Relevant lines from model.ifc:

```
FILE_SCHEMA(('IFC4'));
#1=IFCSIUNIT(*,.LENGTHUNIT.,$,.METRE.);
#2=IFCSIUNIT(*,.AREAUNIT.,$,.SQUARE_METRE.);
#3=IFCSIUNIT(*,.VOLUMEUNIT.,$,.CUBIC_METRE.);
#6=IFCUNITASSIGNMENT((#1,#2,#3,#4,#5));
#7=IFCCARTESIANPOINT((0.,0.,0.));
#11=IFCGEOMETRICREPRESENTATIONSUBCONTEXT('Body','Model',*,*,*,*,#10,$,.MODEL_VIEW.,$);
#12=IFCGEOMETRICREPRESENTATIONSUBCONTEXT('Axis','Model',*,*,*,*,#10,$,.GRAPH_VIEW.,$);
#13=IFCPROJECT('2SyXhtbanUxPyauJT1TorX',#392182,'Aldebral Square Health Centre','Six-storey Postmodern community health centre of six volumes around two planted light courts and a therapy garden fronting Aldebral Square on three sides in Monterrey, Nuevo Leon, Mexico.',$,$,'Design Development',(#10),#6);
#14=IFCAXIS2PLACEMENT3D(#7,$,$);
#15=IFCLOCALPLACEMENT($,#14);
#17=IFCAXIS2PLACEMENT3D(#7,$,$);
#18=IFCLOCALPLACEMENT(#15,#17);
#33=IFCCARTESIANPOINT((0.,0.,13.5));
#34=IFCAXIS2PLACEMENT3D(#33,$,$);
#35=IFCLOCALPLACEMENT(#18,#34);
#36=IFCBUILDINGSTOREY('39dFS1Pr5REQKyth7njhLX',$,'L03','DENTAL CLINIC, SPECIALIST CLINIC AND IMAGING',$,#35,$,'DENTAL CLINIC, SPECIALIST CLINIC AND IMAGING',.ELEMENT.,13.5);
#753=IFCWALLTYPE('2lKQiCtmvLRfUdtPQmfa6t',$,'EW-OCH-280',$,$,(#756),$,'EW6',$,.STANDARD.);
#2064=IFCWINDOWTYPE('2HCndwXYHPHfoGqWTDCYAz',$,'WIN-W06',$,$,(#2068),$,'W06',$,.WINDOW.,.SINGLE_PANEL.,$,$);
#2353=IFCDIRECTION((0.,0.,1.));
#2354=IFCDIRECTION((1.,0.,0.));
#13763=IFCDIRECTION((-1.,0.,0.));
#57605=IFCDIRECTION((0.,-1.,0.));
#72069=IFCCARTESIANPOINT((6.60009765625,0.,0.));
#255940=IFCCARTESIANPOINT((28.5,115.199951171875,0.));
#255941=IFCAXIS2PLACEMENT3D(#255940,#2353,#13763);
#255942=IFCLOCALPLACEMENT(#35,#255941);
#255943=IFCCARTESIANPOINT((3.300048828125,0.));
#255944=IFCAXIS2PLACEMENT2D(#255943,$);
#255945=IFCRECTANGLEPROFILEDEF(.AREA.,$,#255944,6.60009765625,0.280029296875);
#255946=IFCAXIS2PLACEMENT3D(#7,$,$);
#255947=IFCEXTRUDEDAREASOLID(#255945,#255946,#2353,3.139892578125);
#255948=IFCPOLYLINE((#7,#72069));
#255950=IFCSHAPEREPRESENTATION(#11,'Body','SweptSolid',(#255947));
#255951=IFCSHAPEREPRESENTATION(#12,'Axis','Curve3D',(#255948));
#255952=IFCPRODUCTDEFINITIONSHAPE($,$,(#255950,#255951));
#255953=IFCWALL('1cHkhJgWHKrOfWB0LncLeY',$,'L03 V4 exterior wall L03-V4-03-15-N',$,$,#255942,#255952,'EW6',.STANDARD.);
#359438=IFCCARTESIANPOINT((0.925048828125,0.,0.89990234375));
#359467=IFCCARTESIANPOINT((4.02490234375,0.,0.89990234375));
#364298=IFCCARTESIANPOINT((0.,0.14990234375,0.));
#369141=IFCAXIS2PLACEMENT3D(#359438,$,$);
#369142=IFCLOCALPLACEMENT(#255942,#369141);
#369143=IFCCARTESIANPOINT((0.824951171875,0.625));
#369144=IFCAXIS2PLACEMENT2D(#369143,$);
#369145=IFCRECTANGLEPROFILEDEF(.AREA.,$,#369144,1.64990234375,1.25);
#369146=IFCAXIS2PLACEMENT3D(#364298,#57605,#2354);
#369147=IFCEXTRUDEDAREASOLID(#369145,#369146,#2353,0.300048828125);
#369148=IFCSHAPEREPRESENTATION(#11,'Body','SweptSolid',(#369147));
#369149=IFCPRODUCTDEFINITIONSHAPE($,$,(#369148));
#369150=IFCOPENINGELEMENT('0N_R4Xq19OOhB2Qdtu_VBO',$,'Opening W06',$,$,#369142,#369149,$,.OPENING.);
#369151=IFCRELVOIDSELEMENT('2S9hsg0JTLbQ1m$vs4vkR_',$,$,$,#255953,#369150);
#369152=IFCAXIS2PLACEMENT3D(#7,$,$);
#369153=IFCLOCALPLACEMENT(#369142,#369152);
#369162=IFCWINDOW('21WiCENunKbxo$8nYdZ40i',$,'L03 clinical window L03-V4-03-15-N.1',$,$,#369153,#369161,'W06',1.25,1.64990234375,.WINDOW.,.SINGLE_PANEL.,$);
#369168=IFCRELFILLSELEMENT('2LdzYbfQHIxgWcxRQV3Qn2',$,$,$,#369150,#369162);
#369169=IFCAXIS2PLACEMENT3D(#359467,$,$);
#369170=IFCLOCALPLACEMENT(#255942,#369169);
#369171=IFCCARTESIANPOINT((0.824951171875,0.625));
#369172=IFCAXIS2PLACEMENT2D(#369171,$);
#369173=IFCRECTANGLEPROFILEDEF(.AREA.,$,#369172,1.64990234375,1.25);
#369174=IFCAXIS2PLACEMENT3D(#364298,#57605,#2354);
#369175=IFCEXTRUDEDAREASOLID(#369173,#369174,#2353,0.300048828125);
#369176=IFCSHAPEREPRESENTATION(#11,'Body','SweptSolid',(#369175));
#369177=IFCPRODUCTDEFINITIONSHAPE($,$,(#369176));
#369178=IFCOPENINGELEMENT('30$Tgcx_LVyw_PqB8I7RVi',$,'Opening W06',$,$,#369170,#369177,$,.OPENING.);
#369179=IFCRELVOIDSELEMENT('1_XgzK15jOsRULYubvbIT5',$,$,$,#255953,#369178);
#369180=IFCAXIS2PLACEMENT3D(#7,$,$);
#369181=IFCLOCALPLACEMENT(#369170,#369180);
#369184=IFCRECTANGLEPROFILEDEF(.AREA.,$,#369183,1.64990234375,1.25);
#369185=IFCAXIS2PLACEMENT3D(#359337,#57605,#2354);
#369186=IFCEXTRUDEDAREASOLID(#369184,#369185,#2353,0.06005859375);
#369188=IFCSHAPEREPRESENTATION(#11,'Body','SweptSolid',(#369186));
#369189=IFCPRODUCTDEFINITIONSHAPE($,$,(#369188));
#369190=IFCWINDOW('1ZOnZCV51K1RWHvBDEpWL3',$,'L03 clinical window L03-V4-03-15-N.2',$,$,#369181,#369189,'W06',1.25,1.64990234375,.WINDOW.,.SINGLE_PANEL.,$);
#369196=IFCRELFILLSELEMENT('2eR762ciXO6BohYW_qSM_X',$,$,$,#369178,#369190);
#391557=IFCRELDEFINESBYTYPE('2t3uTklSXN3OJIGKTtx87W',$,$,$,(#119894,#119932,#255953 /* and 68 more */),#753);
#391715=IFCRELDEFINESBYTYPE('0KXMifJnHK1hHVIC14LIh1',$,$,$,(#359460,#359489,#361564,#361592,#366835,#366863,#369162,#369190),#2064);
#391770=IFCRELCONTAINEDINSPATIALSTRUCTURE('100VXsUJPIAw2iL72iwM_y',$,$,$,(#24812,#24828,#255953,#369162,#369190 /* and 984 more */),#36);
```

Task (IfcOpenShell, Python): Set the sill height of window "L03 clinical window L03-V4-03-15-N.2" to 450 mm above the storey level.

```python
import numpy as np
import ifcopenshell
import ifcopenshell.api.geometry
import ifcopenshell.geom
import ifcopenshell.util.element
import ifcopenshell.util.placement
import ifcopenshell.util.shape
import ifcopenshell.util.unit

model = ifcopenshell.open("model.ifc")
unit_scale = ifcopenshell.util.unit.calculate_unit_scale(model)

window = model.by_guid("1ZOnZCV51K1RWHvBDEpWL3")
opening = window.FillsVoids[0].RelatingOpeningElement
storey = ifcopenshell.util.element.get_container(window, ifc_class="IfcBuildingStorey")
level = ifcopenshell.util.placement.get_local_placement(storey.ObjectPlacement)[2, 3]

# The opening's origin need not be at the sill, so measure its lowest point.
shape = ifcopenshell.geom.create_shape(ifcopenshell.geom.settings(), opening)
bottom = ifcopenshell.util.shape.get_shape_bottom_elevation(shape, shape.geometry) / unit_scale
dz = level + 0.45 / unit_scale - bottom

shift = np.array([0.0, 0.0, dz])
# The window is placed relative to its opening, so it follows when the opening moves.
matrix = ifcopenshell.util.placement.get_local_placement(opening.ObjectPlacement)
matrix[:3, 3] += shift
ifcopenshell.api.geometry.edit_object_placement(
    model, product=opening, matrix=matrix, is_si=False, should_transform_children=True
)

print(f"moved by {dz * unit_scale:+.3f} m")

model.write("model_v2.ifc")
```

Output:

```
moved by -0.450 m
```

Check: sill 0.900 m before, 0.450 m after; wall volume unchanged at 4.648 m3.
